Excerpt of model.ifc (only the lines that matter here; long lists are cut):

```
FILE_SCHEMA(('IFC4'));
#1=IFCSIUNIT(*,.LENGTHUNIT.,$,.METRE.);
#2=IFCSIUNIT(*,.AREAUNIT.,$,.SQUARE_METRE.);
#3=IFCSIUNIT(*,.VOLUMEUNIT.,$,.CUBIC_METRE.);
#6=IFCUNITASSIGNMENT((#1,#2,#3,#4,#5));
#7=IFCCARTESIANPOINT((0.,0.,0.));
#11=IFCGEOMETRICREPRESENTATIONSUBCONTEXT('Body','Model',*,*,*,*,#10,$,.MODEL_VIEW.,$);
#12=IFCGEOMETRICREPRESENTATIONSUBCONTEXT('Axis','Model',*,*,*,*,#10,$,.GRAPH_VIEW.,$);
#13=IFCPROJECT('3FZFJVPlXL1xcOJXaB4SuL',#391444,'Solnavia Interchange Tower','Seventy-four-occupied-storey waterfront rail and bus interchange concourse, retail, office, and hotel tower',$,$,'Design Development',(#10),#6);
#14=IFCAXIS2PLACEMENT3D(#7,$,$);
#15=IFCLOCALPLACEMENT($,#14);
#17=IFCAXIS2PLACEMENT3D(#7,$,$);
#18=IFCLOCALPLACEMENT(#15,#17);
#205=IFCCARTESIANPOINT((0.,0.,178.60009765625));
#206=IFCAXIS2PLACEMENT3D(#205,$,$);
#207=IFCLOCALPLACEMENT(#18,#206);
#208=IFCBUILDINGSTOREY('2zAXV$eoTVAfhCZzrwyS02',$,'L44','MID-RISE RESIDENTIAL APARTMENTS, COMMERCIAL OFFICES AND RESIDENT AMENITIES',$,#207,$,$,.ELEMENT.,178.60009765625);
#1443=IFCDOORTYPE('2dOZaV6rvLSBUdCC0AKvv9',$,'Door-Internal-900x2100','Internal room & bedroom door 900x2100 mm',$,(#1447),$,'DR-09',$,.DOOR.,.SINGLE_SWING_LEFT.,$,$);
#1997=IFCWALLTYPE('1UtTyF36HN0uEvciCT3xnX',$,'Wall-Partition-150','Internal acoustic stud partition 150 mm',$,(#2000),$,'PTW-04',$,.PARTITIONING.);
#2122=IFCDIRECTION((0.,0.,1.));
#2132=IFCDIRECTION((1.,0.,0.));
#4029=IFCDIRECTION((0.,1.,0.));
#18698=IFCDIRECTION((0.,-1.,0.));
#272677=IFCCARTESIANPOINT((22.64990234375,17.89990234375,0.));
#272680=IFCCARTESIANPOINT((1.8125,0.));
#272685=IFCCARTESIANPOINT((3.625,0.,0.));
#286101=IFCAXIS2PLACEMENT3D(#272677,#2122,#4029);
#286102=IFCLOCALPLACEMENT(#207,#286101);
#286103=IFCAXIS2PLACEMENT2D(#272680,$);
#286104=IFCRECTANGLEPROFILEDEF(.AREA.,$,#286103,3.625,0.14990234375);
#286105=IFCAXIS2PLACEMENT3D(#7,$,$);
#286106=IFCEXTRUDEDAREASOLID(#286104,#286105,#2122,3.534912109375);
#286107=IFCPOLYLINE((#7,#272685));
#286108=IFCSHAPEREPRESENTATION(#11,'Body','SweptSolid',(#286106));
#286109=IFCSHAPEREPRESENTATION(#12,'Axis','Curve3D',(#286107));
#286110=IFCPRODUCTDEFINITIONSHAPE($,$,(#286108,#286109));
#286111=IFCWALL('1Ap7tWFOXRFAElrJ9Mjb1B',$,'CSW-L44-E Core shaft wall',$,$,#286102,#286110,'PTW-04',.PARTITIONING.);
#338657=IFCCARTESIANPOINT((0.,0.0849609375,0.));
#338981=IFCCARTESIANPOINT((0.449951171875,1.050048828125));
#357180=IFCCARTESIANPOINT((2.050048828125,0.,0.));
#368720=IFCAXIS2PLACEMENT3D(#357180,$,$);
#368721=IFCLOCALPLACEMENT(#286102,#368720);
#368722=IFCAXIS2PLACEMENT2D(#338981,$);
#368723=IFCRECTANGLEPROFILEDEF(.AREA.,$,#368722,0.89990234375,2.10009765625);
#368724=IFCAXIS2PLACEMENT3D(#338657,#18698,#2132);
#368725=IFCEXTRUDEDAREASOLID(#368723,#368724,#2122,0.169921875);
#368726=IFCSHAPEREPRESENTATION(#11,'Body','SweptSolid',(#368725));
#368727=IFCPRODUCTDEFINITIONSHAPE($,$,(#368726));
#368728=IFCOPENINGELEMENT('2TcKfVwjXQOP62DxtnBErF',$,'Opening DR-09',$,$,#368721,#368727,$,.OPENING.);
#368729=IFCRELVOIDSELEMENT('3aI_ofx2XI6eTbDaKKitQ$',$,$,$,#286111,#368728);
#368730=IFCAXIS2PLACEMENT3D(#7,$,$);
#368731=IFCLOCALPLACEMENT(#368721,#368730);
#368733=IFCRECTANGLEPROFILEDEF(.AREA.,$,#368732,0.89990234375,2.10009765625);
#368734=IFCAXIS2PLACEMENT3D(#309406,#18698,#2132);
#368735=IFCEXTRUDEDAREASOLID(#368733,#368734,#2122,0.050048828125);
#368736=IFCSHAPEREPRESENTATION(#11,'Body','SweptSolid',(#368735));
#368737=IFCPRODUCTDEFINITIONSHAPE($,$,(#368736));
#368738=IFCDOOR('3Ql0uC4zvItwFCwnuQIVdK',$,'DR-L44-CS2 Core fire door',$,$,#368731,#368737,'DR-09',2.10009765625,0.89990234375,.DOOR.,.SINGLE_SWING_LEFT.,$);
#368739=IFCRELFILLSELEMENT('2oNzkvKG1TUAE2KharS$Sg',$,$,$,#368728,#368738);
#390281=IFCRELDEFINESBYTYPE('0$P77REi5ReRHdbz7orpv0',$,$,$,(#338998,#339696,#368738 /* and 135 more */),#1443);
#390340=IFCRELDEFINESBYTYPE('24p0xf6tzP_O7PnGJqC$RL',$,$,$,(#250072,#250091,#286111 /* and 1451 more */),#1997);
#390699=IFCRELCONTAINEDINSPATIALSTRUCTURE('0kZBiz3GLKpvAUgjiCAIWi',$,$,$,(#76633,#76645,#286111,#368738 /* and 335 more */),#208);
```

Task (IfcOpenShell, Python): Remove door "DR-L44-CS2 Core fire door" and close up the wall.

```python
import ifcopenshell
import ifcopenshell.api.feature
import ifcopenshell.api.root
import ifcopenshell.geom
import ifcopenshell.util.shape

model = ifcopenshell.open("model.ifc")
settings = ifcopenshell.geom.settings()


def volume(element):
    """Net volume in cubic metres, openings subtracted."""
    shape = ifcopenshell.geom.create_shape(settings, element)
    return ifcopenshell.util.shape.get_volume(shape.geometry)


door = model.by_id(368738)
opening = door.FillsVoids[0].RelatingOpeningElement
wall = opening.VoidsElements[0].RelatingBuildingElement
before = volume(wall)

ifcopenshell.api.root.remove_product(model, product=door)
ifcopenshell.api.feature.remove_feature(model, feature=opening)

after = volume(wall)

print(f"wall volume {before:.3f} -> {after:.3f} m3")

model.write("model_v2.ifc")
```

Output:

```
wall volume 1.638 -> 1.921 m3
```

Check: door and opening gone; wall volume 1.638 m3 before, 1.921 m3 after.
